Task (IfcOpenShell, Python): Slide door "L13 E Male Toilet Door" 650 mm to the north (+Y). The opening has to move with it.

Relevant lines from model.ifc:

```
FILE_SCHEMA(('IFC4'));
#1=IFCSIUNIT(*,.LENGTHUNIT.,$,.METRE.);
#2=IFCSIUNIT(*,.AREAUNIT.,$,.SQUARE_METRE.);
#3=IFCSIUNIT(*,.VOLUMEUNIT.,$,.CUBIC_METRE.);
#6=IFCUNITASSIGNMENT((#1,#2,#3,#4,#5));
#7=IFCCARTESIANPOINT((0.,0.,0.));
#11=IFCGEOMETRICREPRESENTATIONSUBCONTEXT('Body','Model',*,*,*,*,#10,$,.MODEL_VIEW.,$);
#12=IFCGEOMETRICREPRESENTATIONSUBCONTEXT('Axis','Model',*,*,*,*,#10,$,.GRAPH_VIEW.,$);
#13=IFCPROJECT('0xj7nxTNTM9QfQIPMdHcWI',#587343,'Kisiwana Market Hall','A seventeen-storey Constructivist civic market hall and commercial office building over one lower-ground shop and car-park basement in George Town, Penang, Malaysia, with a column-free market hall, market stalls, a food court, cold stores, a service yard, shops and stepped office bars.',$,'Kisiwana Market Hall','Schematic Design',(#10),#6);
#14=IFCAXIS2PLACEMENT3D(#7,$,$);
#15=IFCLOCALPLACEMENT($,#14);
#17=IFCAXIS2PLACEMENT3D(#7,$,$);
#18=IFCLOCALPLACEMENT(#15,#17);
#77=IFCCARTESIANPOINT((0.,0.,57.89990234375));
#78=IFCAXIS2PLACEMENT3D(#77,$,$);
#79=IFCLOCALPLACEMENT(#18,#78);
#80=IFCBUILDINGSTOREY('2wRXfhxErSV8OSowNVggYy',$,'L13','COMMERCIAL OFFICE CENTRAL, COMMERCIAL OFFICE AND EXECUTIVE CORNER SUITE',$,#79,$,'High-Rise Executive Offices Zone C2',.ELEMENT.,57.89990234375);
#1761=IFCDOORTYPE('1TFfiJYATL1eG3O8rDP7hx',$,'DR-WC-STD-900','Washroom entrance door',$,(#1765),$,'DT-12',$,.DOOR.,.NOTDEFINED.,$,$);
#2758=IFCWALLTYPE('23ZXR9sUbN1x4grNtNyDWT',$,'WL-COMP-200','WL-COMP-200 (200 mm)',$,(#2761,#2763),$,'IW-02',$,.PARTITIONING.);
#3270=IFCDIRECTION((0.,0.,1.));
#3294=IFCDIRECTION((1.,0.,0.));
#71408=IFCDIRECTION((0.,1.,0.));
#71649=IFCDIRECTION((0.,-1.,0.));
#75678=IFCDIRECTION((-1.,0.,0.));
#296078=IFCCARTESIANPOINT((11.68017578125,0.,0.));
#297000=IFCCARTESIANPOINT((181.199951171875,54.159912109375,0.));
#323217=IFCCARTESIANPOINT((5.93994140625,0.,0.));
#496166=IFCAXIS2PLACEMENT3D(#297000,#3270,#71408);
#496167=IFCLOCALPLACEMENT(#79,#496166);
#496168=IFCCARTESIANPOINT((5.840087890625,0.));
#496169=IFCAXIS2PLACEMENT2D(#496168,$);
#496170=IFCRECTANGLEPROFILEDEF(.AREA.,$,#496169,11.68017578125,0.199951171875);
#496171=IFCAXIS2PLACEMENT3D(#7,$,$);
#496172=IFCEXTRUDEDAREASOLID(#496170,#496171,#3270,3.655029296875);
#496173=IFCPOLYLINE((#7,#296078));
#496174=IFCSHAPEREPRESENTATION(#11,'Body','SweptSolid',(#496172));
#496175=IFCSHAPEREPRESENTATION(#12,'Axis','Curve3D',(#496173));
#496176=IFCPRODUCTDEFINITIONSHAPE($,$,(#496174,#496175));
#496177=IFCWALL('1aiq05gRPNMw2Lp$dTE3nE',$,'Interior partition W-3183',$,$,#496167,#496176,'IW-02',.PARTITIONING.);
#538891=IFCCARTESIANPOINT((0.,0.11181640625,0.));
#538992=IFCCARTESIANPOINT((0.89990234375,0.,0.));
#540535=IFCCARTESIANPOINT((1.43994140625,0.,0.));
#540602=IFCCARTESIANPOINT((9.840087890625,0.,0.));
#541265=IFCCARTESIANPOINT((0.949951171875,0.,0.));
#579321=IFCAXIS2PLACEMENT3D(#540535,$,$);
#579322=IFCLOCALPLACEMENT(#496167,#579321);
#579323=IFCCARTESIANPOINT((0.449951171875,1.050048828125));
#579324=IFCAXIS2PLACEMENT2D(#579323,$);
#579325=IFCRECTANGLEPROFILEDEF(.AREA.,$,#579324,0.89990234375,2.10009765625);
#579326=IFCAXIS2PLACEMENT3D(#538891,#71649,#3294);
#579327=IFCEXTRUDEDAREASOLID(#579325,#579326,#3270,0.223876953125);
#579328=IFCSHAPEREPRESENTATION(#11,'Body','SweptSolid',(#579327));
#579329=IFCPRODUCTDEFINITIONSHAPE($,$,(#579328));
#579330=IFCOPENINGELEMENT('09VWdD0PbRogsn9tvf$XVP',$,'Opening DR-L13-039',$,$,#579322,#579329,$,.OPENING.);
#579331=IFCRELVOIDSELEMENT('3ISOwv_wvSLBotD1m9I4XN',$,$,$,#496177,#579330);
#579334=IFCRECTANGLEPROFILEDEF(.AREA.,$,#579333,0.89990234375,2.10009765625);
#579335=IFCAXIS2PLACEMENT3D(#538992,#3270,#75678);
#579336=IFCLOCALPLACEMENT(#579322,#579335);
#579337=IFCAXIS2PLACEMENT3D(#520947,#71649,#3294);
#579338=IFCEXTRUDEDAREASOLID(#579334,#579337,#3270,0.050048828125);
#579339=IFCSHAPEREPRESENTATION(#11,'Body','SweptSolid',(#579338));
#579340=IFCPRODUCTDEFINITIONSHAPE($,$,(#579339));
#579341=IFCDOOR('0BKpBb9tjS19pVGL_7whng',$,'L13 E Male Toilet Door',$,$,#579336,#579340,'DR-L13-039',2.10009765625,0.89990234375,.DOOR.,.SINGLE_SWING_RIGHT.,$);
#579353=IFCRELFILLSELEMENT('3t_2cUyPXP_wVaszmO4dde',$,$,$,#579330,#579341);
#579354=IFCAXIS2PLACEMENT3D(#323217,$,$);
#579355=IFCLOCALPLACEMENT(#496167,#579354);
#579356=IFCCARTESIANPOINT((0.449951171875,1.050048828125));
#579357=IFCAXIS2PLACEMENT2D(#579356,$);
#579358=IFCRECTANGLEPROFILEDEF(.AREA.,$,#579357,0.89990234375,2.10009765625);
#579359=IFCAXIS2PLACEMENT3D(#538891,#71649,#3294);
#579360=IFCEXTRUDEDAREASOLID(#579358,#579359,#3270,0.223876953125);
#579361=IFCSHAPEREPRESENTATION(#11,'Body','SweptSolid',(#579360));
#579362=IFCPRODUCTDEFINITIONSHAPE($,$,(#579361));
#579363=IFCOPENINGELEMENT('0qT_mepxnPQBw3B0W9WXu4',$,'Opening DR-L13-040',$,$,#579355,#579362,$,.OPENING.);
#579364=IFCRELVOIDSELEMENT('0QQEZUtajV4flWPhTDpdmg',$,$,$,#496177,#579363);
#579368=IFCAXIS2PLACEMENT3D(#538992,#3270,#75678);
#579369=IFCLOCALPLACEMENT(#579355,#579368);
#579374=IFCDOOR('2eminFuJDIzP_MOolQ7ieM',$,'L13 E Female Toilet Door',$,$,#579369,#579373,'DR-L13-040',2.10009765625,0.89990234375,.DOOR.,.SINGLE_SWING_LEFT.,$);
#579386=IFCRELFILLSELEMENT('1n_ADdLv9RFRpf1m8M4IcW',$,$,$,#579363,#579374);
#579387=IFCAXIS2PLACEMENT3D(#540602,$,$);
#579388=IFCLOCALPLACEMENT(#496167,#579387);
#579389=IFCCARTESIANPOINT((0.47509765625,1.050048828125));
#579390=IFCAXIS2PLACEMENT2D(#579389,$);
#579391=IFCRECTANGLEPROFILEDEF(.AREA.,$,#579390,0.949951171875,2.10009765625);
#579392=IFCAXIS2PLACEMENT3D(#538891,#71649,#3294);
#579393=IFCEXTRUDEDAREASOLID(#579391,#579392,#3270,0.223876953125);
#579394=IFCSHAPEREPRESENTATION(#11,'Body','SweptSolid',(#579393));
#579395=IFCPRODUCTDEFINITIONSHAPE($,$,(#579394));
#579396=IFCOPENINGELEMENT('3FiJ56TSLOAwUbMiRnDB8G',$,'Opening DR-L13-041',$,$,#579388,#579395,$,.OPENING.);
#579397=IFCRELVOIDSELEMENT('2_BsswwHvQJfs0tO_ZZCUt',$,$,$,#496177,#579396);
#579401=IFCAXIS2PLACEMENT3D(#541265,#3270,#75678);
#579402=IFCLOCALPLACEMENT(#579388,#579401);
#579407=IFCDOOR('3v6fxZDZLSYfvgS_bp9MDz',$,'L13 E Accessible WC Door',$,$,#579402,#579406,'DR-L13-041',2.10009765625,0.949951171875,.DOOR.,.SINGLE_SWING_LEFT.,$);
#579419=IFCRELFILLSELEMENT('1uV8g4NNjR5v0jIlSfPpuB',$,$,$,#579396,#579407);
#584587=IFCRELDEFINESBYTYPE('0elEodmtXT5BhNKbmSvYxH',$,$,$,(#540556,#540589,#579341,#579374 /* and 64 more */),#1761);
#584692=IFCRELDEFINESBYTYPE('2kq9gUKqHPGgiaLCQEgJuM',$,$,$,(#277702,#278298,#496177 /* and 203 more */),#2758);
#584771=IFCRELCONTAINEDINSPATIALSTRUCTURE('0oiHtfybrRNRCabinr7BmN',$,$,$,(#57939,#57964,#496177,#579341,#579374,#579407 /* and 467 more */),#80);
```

```python
import ifcopenshell
import ifcopenshell.api.geometry
import ifcopenshell.util.placement
import ifcopenshell.util.unit

model = ifcopenshell.open("model.ifc")
unit_scale = ifcopenshell.util.unit.calculate_unit_scale(model)

door = model.by_guid("0BKpBb9tjS19pVGL_7whng")
opening = door.FillsVoids[0].RelatingOpeningElement
wall = opening.VoidsElements[0].RelatingBuildingElement

wall_matrix = ifcopenshell.util.placement.get_local_placement(wall.ObjectPlacement)
shift = wall_matrix[:3, 0] * 0.65 / unit_scale
before = ifcopenshell.util.placement.get_local_placement(door.ObjectPlacement)[:3, 3].copy()

# The door is placed relative to its opening, so it follows when the opening moves.
matrix = ifcopenshell.util.placement.get_local_placement(opening.ObjectPlacement)
matrix[:3, 3] += shift
ifcopenshell.api.geometry.edit_object_placement(
    model, product=opening, matrix=matrix, is_si=False, should_transform_children=True
)

after = ifcopenshell.util.placement.get_local_placement(door.ObjectPlacement)[:3, 3]
print("door moved by", (after - before).round(3) + 0.0)

model.write("model_edited.ifc")
```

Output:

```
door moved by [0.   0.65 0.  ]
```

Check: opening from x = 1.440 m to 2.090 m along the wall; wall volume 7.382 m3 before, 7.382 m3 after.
